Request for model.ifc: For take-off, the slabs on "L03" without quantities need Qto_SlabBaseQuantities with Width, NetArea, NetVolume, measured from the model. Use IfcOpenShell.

First a look at what the model holds.

```python
import ifcopenshell
import ifcopenshell.util.element
import ifcopenshell.util.unit

model = ifcopenshell.open("model.ifc")
print(model.schema)
for unit_type in ("LENGTHUNIT", "AREAUNIT", "VOLUMEUNIT"):
    print(unit_type, ifcopenshell.util.unit.calculate_unit_scale(model, unit_type))
storey = next(s for s in model.by_type("IfcBuildingStorey") if s.Name == "L03")
slabs = [e for e in ifcopenshell.util.element.get_decomposition(storey) if e.is_a("IfcSlab")]
for e in sorted(slabs, key=lambda e: e.id()):
    print(e.id(), e.is_a(), e.Name, list(ifcopenshell.util.element.get_psets(e, qtos_only=True)), sep=" | ")
```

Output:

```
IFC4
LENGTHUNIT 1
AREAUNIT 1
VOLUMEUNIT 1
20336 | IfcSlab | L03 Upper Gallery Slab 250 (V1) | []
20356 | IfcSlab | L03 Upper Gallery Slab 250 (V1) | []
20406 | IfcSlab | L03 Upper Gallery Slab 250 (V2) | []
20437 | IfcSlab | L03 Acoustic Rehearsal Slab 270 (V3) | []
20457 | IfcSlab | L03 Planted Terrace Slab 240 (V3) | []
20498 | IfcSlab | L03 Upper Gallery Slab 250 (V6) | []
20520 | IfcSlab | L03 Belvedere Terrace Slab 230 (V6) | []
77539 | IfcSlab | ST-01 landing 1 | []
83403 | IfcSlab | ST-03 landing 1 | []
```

```python
import ifcopenshell
import ifcopenshell.api.pset
import ifcopenshell.geom
import ifcopenshell.util.element
import ifcopenshell.util.shape
import ifcopenshell.util.unit

model = ifcopenshell.open("model.ifc")
unit_scale = ifcopenshell.util.unit.calculate_unit_scale(model)
area_scale = ifcopenshell.util.unit.calculate_unit_scale(model, "AREAUNIT")
volume_scale = ifcopenshell.util.unit.calculate_unit_scale(model, "VOLUMEUNIT")
settings = ifcopenshell.geom.settings()

storey = next(s for s in model.by_type("IfcBuildingStorey") if s.Name == "L03")
slabs = [e for e in ifcopenshell.util.element.get_decomposition(storey) if e.is_a("IfcSlab")]

for e in sorted(slabs, key=lambda e: e.id()):
    if ifcopenshell.util.element.get_psets(e, qtos_only=True, should_inherit=False):
        continue
    # Geometry comes back in metres, in the element's own axes.
    shape = ifcopenshell.geom.create_shape(settings, e)
    values = {
        "Width": ifcopenshell.util.shape.get_z(shape.geometry) / unit_scale,
        "NetArea": ifcopenshell.util.shape.get_footprint_area(shape.geometry) / area_scale,
        "NetVolume": ifcopenshell.util.shape.get_volume(shape.geometry) / volume_scale,
    }
    qto = ifcopenshell.api.pset.add_qto(model, product=e, name="Qto_SlabBaseQuantities")
    ifcopenshell.api.pset.edit_qto(model, qto=qto, properties=values)
    print(e.id(), {k: round(v, 3) for k, v in values.items()})

model.write("model-out.ifc")
```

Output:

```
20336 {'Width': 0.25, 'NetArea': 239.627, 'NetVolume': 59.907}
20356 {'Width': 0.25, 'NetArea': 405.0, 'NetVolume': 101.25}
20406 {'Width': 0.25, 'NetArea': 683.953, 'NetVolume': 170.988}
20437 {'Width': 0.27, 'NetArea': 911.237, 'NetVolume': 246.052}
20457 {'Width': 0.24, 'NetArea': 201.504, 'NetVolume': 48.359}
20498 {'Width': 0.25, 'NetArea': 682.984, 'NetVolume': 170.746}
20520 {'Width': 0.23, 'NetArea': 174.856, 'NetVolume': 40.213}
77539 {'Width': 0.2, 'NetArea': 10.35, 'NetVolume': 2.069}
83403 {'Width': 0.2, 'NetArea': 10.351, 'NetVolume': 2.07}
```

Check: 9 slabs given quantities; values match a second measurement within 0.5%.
